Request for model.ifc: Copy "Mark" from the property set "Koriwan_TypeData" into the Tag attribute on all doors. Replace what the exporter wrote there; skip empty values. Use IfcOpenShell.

First a look at what the model holds.

```python
import ifcopenshell
import ifcopenshell.util.element

model = ifcopenshell.open("model.ifc")
print(model.schema)
doors = model.by_type("IfcDoor")
print(len(doors), "doors")
for e in doors[:8]:
    source = ifcopenshell.util.element.get_pset(e, "Koriwan_TypeData", "Mark")
    target = e.Tag
    print(e.id(), repr(source), repr(target), sep=" | ")
```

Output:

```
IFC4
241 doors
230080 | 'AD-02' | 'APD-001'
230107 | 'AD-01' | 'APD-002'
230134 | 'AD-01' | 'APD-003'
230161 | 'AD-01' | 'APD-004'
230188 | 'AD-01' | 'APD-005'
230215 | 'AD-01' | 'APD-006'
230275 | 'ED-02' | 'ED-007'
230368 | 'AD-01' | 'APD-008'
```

```python
import ifcopenshell
import ifcopenshell.util.element

model = ifcopenshell.open("model.ifc")

count = 0
for e in model.by_type("IfcDoor"):
    value = ifcopenshell.util.element.get_pset(e, "Koriwan_TypeData", "Mark")
    current = e.Tag
    if not value or not value.strip() or current == value:
        continue
    e.Tag = value
    count += 1

print(count, "doors updated")

model.write("model_edited.ifc")
```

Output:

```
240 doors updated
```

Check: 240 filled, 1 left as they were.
